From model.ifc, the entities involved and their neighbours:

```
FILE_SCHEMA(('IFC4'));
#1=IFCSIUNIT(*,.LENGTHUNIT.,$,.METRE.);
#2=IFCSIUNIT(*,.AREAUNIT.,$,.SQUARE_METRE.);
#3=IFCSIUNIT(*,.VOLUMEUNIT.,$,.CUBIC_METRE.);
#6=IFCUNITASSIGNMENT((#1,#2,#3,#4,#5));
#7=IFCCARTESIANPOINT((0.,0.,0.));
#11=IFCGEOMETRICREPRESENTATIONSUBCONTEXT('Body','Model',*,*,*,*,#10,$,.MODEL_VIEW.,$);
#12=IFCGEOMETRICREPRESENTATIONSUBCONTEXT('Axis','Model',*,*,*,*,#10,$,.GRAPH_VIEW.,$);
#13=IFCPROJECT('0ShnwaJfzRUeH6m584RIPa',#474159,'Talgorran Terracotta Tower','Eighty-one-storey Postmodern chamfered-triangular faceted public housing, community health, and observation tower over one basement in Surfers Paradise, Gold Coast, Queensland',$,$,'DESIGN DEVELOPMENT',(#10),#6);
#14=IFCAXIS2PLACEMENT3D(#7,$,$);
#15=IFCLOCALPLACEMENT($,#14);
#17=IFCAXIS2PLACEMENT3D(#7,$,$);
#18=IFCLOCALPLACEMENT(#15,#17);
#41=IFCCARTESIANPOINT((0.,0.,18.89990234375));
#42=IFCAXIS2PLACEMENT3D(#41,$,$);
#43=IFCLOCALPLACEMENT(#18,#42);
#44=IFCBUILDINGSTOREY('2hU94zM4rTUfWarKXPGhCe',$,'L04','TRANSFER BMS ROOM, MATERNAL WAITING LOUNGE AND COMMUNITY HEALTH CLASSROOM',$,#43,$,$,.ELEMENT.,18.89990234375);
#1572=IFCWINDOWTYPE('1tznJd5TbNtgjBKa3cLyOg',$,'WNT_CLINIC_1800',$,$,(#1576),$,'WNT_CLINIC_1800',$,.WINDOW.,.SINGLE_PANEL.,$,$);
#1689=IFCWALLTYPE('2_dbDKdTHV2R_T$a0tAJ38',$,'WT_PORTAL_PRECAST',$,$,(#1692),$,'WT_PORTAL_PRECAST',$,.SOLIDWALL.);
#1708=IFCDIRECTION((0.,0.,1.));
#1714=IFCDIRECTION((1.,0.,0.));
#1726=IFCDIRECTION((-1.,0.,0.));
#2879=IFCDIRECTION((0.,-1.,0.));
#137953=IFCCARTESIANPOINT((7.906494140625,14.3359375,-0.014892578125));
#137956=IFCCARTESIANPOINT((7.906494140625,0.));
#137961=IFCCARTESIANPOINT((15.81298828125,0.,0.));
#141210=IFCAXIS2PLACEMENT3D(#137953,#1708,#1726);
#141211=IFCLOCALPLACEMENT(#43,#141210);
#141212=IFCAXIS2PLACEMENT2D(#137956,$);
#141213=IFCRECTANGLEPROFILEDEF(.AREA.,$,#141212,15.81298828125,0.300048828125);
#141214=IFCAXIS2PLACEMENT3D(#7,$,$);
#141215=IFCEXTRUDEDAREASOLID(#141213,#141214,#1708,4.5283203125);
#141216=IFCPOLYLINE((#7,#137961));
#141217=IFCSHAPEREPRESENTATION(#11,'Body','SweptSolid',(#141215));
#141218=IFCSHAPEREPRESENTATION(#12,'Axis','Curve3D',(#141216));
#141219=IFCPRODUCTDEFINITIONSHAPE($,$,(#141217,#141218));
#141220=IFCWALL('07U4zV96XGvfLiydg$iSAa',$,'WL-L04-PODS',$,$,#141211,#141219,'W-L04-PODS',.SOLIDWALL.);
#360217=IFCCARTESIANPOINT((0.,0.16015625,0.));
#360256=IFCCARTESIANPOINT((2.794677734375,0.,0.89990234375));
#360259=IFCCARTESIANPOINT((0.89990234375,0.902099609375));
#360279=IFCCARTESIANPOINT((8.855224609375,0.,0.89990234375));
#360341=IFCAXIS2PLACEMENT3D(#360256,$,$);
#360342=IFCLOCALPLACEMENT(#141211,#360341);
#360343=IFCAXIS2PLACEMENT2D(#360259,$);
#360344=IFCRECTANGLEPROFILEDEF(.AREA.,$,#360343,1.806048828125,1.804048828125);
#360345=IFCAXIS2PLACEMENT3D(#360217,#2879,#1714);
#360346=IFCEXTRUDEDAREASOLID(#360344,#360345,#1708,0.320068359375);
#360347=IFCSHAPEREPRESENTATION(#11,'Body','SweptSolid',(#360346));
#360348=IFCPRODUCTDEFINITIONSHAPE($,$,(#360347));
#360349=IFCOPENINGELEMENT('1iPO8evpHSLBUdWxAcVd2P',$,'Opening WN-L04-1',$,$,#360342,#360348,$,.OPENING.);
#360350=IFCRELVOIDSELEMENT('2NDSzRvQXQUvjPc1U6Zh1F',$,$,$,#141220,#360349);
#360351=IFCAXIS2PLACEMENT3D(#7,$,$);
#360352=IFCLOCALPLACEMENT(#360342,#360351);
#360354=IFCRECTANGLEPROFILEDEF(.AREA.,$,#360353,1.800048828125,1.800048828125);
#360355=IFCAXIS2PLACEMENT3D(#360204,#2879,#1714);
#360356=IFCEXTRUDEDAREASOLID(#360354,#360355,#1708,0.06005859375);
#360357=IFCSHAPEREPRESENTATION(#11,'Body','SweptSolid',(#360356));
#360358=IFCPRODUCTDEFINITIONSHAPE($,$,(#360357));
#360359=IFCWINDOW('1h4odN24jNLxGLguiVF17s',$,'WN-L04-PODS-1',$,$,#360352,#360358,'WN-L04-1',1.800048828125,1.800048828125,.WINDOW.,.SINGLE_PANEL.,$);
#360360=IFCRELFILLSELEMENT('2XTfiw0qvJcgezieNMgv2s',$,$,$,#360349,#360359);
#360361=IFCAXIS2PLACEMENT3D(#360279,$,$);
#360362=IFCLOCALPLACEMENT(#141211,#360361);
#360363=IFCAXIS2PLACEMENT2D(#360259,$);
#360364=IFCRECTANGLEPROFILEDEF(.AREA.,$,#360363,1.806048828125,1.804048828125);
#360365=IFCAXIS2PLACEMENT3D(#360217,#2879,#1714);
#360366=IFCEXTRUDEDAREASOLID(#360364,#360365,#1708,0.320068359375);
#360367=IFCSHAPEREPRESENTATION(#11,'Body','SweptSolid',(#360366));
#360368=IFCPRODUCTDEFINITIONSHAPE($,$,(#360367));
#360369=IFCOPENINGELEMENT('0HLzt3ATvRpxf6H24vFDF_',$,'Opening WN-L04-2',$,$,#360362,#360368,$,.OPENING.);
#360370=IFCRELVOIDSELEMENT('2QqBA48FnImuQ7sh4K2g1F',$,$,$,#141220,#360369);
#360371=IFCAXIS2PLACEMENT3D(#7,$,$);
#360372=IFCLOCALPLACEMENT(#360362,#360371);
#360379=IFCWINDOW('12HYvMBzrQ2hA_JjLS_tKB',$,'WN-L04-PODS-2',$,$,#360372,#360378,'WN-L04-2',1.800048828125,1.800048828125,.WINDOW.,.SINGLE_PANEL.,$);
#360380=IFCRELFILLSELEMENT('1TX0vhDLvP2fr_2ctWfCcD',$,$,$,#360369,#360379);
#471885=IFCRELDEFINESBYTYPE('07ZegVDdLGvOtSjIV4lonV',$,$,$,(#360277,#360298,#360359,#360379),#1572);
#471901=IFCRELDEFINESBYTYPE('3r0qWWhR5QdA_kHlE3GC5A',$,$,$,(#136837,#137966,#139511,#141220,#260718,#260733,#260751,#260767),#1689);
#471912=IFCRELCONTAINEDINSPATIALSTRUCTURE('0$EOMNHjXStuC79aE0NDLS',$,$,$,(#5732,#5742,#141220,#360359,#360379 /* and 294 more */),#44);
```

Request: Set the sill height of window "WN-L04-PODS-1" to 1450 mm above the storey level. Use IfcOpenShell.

```python
import numpy as np
import ifcopenshell
import ifcopenshell.api.geometry
import ifcopenshell.geom
import ifcopenshell.util.element
import ifcopenshell.util.placement
import ifcopenshell.util.shape
import ifcopenshell.util.unit

model = ifcopenshell.open("model.ifc")
unit_scale = ifcopenshell.util.unit.calculate_unit_scale(model)

window = model.by_guid("1h4odN24jNLxGLguiVF17s")
opening = window.FillsVoids[0].RelatingOpeningElement
storey = ifcopenshell.util.element.get_container(window, ifc_class="IfcBuildingStorey")
level = ifcopenshell.util.placement.get_local_placement(storey.ObjectPlacement)[2, 3]

# The opening's origin need not be at the sill, so measure its lowest point.
shape = ifcopenshell.geom.create_shape(ifcopenshell.geom.settings(), opening)
bottom = ifcopenshell.util.shape.get_shape_bottom_elevation(shape, shape.geometry) / unit_scale
dz = level + 1.45 - bottom

shift = np.array([0.0, 0.0, dz])
# The window is placed relative to its opening, so it follows when the opening moves.
matrix = ifcopenshell.util.placement.get_local_placement(opening.ObjectPlacement)
matrix[:3, 3] += shift
ifcopenshell.api.geometry.edit_object_placement(
    model, product=opening, matrix=matrix, is_si=False, should_transform_children=True
)

print(f"moved by {dz * unit_scale:+.3f} m")

model.write("model_edited.ifc")
```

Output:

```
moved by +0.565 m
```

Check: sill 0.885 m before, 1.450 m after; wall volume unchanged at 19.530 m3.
